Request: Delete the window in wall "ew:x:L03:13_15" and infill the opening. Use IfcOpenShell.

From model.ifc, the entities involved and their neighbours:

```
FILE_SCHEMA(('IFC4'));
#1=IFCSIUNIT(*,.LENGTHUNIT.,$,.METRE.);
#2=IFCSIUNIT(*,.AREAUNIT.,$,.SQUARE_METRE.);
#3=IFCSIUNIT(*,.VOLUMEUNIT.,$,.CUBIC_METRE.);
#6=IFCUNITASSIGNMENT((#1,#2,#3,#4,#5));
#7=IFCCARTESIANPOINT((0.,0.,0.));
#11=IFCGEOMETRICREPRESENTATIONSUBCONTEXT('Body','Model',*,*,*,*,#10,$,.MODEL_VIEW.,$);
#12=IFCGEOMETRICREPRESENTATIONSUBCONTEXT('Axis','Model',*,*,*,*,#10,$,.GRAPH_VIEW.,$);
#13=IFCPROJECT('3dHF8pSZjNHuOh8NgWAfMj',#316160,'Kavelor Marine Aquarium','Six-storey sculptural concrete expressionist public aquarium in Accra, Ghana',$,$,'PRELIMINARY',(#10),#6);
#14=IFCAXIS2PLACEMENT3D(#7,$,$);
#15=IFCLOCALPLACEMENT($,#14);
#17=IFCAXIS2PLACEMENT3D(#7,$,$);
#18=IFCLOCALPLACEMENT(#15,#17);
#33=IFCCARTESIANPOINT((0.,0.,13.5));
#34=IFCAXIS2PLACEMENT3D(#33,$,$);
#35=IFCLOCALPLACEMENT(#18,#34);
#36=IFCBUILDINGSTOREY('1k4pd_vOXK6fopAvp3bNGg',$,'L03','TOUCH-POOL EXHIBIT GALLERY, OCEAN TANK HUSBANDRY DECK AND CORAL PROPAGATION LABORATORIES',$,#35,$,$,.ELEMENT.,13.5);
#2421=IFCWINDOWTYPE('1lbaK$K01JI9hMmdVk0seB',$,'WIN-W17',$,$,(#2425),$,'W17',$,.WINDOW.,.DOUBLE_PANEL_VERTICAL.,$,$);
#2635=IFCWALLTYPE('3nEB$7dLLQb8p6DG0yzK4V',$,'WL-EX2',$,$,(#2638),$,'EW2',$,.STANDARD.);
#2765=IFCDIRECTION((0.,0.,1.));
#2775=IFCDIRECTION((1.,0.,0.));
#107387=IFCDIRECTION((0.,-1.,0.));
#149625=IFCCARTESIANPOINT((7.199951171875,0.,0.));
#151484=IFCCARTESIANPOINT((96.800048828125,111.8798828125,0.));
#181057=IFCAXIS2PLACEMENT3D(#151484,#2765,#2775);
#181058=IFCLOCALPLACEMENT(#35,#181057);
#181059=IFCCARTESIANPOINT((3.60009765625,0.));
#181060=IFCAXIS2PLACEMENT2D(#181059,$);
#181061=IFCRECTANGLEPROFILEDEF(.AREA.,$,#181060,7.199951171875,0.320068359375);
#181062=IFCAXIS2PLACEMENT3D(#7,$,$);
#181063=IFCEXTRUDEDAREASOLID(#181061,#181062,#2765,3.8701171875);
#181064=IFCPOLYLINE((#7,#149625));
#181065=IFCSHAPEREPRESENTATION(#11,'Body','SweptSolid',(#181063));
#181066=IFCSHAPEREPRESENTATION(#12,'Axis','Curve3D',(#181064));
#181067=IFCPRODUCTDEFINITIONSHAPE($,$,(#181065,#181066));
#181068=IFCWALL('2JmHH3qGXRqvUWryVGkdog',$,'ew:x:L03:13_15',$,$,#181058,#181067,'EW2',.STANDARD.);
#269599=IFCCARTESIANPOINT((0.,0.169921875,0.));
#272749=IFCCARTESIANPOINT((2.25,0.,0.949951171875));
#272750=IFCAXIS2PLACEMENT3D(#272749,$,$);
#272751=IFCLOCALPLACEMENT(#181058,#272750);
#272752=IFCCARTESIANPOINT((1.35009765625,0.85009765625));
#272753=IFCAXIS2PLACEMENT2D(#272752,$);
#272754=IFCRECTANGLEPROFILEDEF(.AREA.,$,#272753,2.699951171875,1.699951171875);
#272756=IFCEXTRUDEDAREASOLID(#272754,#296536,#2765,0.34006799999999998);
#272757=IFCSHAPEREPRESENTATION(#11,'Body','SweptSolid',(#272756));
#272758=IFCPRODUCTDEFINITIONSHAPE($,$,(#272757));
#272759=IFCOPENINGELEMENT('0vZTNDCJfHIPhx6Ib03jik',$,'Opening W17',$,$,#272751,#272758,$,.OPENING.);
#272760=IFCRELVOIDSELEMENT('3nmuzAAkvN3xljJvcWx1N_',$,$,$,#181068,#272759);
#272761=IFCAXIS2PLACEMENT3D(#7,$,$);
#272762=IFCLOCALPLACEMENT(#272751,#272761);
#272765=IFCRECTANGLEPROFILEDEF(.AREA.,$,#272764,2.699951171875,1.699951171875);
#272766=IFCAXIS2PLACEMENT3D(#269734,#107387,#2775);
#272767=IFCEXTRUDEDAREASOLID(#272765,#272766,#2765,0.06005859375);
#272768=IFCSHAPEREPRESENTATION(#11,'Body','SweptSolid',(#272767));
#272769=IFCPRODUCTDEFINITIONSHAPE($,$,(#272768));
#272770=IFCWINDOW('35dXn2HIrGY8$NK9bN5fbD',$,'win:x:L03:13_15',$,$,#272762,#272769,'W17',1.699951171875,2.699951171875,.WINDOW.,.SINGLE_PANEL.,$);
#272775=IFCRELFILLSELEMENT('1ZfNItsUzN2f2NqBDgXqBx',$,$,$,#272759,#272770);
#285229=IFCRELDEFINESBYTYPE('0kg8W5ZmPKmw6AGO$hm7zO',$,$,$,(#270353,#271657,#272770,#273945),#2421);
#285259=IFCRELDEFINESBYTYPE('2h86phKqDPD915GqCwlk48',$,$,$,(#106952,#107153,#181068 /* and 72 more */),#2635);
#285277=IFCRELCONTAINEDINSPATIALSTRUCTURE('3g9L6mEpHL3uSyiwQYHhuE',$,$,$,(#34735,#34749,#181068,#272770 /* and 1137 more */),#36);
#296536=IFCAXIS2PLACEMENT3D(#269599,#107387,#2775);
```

```python
import ifcopenshell
import ifcopenshell.api.feature
import ifcopenshell.api.root
import ifcopenshell.geom
import ifcopenshell.util.shape

model = ifcopenshell.open("model.ifc")
settings = ifcopenshell.geom.settings()


def volume(element):
    """Net volume in cubic metres, openings subtracted."""
    shape = ifcopenshell.geom.create_shape(settings, element)
    return ifcopenshell.util.shape.get_volume(shape.geometry)


window = model.by_guid("35dXn2HIrGY8$NK9bN5fbD")
opening = window.FillsVoids[0].RelatingOpeningElement
wall = opening.VoidsElements[0].RelatingBuildingElement
before = volume(wall)

ifcopenshell.api.root.remove_product(model, product=window)
ifcopenshell.api.feature.remove_feature(model, feature=opening)

after = volume(wall)

print(f"wall volume {before:.3f} -> {after:.3f} m3")

model.write("model_v2.ifc")
```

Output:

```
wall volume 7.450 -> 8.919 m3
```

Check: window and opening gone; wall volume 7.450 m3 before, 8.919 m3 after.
